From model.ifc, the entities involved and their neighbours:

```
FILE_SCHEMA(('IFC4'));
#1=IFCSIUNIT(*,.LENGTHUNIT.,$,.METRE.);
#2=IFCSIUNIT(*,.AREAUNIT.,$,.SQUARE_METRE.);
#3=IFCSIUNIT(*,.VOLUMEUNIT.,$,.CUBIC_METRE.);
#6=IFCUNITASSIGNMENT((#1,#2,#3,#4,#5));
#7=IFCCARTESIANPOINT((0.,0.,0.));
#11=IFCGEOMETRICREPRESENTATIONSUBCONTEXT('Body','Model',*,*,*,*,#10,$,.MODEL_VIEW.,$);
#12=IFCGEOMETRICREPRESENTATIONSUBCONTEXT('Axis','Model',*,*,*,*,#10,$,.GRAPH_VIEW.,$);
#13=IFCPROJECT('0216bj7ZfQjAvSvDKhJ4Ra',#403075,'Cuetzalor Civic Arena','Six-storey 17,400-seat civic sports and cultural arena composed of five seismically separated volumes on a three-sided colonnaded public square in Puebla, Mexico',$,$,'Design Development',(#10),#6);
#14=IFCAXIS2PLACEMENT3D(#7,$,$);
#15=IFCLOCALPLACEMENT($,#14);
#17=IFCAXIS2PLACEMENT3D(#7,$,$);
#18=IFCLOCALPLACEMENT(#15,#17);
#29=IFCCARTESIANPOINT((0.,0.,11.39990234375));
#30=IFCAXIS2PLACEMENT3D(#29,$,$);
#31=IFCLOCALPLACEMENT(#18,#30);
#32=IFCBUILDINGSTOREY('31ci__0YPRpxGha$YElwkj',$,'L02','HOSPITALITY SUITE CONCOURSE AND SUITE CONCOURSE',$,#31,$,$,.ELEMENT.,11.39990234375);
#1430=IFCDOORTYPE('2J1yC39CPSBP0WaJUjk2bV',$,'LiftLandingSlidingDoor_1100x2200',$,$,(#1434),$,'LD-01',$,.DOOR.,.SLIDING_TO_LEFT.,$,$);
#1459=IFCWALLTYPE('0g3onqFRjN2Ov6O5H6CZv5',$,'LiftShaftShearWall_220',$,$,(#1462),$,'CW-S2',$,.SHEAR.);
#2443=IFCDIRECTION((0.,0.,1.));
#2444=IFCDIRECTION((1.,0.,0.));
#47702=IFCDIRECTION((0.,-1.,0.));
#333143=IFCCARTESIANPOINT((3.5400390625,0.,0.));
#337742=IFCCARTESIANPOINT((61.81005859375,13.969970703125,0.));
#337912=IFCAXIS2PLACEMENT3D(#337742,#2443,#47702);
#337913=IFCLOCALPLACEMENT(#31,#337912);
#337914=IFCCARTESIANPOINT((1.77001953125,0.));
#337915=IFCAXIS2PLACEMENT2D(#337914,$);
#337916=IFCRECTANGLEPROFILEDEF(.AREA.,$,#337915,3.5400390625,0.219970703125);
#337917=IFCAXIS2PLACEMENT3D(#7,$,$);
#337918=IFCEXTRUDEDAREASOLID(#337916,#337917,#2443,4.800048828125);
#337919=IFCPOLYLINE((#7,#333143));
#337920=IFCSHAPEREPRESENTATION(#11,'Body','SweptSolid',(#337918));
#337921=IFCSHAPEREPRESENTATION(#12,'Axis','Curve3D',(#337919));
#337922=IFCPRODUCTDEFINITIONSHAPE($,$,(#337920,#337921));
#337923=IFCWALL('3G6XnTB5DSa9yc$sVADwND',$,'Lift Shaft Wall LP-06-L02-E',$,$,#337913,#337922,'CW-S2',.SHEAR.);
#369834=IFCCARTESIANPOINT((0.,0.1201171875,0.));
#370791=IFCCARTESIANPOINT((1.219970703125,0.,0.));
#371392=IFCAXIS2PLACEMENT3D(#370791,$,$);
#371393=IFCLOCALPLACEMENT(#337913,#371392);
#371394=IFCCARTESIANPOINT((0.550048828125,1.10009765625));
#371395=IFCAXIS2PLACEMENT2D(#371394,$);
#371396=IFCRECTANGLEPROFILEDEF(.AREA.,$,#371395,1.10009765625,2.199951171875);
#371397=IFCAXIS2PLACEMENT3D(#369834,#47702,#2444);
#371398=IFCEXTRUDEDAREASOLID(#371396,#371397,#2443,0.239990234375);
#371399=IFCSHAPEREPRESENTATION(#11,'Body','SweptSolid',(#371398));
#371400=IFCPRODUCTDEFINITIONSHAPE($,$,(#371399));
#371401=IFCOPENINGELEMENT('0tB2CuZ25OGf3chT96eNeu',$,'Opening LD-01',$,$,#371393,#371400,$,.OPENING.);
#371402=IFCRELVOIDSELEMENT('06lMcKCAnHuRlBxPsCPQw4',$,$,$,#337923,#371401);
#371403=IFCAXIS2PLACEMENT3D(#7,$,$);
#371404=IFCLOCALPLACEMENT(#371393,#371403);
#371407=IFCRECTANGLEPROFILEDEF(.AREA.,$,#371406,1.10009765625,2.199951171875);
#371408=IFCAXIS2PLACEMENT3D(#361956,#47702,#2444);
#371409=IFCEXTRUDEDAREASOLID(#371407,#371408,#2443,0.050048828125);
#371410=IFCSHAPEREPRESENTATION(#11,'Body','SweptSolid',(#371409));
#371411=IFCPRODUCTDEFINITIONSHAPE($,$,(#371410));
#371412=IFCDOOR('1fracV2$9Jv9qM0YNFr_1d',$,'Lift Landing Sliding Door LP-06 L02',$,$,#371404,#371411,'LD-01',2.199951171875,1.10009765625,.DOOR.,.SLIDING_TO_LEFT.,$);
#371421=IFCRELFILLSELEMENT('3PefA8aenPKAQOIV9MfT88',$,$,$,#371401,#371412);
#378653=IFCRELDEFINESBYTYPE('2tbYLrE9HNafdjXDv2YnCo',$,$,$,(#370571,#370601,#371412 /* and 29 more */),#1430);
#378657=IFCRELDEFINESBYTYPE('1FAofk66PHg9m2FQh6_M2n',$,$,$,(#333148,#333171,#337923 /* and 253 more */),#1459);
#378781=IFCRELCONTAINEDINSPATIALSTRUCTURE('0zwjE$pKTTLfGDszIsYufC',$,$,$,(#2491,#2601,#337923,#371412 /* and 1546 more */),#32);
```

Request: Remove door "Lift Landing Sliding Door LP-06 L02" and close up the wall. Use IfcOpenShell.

```python
import ifcopenshell
import ifcopenshell.api.feature
import ifcopenshell.api.root
import ifcopenshell.geom
import ifcopenshell.util.shape

model = ifcopenshell.open("model.ifc")
settings = ifcopenshell.geom.settings()


def volume(element):
    """Net volume in cubic metres, openings subtracted."""
    shape = ifcopenshell.geom.create_shape(settings, element)
    return ifcopenshell.util.shape.get_volume(shape.geometry)


door = model.by_guid("1fracV2$9Jv9qM0YNFr_1d")
opening = door.FillsVoids[0].RelatingOpeningElement
wall = opening.VoidsElements[0].RelatingBuildingElement
before = volume(wall)

ifcopenshell.api.root.remove_product(model, product=door)
ifcopenshell.api.feature.remove_feature(model, feature=opening)

after = volume(wall)

print(f"wall volume {before:.3f} -> {after:.3f} m3")

model.write("model_rev.ifc")
```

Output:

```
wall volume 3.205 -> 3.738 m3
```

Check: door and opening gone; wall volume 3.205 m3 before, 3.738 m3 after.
